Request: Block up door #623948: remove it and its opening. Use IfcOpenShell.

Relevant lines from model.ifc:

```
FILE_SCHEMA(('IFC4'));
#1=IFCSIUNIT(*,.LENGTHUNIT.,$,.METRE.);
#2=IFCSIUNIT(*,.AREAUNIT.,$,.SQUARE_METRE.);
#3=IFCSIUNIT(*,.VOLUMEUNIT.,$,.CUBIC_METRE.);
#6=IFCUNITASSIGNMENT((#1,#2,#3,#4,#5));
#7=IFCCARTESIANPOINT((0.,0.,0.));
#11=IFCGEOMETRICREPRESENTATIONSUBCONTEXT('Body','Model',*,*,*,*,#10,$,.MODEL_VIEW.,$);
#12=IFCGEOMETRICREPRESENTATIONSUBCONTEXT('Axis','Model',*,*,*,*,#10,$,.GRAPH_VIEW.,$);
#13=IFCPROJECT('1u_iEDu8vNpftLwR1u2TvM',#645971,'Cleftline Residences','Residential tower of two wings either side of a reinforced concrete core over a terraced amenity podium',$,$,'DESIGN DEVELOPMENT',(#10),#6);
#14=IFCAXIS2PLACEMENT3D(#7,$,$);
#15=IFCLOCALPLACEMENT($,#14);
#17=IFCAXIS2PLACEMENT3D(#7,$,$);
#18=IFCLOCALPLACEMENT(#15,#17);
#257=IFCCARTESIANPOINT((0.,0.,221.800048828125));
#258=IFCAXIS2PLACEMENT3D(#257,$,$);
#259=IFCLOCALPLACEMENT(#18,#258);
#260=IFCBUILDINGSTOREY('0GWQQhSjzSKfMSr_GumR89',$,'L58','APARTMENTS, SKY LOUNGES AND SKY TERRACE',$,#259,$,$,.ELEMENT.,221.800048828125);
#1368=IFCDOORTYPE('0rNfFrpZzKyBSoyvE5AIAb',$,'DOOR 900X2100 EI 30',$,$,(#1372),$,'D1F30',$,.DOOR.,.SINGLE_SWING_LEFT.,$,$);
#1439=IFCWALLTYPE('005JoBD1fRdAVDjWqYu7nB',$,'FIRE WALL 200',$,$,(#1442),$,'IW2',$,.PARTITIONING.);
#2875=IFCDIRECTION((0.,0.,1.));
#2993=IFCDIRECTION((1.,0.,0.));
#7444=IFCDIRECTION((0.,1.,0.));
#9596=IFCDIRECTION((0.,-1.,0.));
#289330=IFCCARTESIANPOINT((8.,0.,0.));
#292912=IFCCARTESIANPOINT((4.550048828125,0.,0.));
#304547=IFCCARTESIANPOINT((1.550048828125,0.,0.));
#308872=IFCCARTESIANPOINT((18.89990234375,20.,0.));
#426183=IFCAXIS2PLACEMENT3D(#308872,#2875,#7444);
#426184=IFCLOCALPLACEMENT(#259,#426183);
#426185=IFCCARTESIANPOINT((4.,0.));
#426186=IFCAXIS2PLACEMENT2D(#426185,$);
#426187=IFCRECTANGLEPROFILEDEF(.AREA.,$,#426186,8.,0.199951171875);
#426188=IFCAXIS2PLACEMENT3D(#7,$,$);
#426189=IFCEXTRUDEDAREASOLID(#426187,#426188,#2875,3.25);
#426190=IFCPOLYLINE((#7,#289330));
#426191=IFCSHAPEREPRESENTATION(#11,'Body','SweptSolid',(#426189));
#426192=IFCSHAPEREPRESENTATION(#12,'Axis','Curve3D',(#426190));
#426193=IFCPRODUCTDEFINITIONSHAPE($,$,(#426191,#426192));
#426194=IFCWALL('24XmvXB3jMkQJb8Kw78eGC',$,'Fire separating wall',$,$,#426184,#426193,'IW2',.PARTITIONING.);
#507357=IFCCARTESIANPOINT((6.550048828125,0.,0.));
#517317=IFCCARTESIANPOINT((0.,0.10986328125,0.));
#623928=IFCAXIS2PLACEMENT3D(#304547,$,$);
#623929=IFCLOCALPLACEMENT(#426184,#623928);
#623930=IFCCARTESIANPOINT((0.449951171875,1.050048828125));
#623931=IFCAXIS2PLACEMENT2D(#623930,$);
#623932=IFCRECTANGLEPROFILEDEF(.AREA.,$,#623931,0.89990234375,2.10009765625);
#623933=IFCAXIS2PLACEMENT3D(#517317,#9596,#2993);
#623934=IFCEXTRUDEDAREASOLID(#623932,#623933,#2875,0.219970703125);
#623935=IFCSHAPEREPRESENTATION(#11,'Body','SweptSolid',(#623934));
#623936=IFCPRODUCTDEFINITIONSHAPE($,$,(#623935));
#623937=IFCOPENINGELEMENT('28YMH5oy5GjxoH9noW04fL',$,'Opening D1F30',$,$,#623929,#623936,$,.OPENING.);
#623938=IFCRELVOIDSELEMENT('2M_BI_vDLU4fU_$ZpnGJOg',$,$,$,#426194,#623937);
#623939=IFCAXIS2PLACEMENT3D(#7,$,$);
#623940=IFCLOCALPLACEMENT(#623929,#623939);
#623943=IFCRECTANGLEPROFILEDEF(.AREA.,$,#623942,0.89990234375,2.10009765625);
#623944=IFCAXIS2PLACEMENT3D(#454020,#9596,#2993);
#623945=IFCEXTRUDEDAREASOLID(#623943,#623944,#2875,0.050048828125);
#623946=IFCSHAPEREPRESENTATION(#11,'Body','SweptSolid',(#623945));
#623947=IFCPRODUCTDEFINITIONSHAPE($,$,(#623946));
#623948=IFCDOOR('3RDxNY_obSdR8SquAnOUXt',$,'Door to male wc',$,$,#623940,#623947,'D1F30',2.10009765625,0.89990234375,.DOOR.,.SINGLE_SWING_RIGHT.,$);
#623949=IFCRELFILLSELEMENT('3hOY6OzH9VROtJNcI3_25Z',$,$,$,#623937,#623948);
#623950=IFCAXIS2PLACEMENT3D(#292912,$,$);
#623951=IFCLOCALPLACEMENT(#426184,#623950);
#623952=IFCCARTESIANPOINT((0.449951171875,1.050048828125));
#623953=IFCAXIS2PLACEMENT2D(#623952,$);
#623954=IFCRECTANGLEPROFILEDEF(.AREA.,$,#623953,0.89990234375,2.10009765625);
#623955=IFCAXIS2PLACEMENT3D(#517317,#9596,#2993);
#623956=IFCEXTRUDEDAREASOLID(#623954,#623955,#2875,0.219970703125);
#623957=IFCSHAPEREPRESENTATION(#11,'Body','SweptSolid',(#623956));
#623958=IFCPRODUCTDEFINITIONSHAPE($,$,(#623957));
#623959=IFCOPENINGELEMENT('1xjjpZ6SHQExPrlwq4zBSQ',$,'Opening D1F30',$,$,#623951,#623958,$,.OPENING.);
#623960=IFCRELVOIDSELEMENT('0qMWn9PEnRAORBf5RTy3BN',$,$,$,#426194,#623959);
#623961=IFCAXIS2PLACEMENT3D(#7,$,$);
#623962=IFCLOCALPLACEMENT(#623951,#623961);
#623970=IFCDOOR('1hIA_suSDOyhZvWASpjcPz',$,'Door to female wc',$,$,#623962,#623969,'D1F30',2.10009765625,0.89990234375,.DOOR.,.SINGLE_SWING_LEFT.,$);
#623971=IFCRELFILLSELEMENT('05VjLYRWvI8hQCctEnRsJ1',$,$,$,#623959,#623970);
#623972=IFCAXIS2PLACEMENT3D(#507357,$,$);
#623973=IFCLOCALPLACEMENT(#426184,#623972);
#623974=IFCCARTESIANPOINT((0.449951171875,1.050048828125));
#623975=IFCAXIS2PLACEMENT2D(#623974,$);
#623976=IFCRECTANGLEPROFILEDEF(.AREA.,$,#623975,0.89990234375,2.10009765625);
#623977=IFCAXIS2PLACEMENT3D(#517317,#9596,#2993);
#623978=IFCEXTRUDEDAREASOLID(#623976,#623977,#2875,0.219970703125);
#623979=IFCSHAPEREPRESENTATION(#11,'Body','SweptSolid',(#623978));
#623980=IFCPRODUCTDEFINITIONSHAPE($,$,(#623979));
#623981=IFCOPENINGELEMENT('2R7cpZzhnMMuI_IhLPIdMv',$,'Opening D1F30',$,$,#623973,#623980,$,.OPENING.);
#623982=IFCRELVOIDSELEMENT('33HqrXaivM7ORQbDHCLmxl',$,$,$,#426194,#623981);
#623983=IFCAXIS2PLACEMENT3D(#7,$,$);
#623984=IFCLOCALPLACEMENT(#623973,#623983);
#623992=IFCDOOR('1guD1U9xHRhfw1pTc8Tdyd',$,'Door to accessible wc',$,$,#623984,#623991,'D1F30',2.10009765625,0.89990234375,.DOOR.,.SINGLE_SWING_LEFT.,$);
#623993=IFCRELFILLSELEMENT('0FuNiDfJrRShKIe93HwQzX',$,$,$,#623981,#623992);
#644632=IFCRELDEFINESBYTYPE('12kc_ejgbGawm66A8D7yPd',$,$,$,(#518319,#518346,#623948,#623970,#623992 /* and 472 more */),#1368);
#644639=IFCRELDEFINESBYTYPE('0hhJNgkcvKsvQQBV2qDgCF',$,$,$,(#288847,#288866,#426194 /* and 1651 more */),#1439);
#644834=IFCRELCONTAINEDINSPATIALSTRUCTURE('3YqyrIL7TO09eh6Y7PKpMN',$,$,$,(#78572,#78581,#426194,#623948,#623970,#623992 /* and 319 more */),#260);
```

```python
import ifcopenshell
import ifcopenshell.api.feature
import ifcopenshell.api.root
import ifcopenshell.geom
import ifcopenshell.util.shape

model = ifcopenshell.open("model.ifc")
settings = ifcopenshell.geom.settings()


def volume(element):
    """Net volume in cubic metres, openings subtracted."""
    shape = ifcopenshell.geom.create_shape(settings, element)
    return ifcopenshell.util.shape.get_volume(shape.geometry)


door = model.by_guid("3RDxNY_obSdR8SquAnOUXt")
opening = door.FillsVoids[0].RelatingOpeningElement
wall = opening.VoidsElements[0].RelatingBuildingElement
before = volume(wall)

ifcopenshell.api.root.remove_product(model, product=door)
ifcopenshell.api.feature.remove_feature(model, feature=opening)

after = volume(wall)

print(f"wall volume {before:.3f} -> {after:.3f} m3")

model.write("model_v2.ifc")
```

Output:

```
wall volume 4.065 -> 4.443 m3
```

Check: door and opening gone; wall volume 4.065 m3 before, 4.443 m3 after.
